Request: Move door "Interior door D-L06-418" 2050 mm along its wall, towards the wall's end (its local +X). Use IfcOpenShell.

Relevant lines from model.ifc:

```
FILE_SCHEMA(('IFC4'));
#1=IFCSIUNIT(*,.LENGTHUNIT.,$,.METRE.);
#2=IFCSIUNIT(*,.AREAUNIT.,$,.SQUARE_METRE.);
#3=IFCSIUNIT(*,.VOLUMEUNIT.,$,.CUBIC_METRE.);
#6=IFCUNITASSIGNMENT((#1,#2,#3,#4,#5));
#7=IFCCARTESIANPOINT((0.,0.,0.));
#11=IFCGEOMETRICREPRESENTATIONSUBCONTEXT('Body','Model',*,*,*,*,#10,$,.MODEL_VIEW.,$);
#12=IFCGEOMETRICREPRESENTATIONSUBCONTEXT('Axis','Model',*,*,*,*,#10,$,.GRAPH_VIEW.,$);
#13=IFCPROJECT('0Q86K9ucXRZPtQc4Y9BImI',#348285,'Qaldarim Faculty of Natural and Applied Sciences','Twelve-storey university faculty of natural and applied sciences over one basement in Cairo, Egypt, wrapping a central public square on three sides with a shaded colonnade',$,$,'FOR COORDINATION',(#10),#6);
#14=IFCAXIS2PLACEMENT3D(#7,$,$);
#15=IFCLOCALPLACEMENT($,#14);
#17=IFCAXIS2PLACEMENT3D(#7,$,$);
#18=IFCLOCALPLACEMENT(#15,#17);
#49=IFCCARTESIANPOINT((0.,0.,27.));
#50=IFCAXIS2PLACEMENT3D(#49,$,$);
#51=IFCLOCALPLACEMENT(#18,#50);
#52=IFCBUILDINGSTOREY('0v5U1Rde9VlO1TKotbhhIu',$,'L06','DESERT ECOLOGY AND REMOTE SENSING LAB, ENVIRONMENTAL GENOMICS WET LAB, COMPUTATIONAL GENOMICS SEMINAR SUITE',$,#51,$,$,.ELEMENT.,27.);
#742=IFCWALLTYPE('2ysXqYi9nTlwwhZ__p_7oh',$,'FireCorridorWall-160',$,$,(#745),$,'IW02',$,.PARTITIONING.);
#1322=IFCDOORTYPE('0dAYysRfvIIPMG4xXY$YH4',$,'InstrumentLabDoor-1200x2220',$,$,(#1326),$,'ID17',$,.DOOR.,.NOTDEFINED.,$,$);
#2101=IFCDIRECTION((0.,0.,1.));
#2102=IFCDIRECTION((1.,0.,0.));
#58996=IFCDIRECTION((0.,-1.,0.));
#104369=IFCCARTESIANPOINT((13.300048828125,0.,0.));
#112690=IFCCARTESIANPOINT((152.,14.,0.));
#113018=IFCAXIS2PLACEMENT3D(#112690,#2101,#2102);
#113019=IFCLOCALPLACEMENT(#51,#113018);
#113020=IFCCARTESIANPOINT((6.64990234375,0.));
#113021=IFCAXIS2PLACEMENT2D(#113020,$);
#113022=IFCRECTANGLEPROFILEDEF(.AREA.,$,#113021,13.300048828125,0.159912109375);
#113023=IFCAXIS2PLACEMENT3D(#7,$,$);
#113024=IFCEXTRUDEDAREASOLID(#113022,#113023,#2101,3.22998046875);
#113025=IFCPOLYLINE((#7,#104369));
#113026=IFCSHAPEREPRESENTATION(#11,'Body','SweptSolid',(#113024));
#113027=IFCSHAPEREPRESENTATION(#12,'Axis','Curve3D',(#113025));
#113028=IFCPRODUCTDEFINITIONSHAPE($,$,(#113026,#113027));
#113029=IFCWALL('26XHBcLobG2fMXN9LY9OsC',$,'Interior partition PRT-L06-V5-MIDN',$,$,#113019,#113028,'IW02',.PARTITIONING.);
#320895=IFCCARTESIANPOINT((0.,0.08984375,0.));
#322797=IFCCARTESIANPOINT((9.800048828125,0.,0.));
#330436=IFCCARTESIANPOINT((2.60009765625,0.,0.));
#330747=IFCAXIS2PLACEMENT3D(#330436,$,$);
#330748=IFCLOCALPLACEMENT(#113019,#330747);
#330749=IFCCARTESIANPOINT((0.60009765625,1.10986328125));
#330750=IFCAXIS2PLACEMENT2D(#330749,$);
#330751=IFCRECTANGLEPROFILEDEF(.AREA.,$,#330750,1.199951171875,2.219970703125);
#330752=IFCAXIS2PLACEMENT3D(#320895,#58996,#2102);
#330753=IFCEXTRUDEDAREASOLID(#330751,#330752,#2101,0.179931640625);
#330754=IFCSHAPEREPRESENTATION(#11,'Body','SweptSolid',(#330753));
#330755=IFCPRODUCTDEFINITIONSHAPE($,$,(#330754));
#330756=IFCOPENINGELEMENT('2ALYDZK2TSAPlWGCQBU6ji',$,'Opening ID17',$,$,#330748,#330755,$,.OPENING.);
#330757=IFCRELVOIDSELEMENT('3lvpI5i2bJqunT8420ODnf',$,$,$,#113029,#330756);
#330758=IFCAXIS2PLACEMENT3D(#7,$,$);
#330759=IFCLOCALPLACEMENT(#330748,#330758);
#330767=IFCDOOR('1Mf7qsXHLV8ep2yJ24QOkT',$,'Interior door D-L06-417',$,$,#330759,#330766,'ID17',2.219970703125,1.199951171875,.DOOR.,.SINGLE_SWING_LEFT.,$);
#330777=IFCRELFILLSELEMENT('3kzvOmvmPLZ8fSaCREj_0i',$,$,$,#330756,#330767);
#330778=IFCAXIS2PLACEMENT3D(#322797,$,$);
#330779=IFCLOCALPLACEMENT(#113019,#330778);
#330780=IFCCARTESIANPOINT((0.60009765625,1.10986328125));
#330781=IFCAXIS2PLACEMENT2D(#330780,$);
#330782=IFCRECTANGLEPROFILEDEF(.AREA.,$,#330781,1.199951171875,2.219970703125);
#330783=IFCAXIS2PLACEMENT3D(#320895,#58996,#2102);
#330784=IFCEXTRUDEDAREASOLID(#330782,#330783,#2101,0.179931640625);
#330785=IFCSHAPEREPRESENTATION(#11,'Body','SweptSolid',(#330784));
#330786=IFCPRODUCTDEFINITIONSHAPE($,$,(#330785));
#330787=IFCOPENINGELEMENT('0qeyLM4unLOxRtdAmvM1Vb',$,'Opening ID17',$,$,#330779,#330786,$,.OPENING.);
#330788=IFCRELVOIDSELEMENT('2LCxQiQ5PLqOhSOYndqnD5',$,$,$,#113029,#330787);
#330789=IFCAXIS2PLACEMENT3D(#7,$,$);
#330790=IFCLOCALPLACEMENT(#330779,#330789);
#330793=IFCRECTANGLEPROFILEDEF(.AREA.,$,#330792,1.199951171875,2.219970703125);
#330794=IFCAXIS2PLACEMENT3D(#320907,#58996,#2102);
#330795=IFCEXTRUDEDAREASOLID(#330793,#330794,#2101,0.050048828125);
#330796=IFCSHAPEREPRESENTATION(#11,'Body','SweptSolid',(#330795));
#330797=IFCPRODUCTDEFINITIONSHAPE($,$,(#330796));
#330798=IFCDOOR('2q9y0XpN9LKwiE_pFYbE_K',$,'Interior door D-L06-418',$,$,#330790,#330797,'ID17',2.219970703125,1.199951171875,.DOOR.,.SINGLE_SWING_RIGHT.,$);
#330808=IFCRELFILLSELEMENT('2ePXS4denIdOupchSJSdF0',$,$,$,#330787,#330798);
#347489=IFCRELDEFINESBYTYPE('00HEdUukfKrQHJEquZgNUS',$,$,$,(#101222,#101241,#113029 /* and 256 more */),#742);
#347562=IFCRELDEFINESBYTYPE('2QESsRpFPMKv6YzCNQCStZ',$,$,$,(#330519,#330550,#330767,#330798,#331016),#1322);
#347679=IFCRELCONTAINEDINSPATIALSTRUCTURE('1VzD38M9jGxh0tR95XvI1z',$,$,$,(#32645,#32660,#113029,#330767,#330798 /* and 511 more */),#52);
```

```python
import ifcopenshell
import ifcopenshell.api.geometry
import ifcopenshell.util.placement

model = ifcopenshell.open("model.ifc")

door = model.by_guid("2q9y0XpN9LKwiE_pFYbE_K")
opening = door.FillsVoids[0].RelatingOpeningElement
wall = opening.VoidsElements[0].RelatingBuildingElement

wall_matrix = ifcopenshell.util.placement.get_local_placement(wall.ObjectPlacement)
shift = wall_matrix[:3, 0] * 2.05
before = ifcopenshell.util.placement.get_local_placement(door.ObjectPlacement)[:3, 3].copy()

# The door is placed relative to its opening, so it follows when the opening moves.
matrix = ifcopenshell.util.placement.get_local_placement(opening.ObjectPlacement)
matrix[:3, 3] += shift
ifcopenshell.api.geometry.edit_object_placement(
    model, product=opening, matrix=matrix, is_si=False, should_transform_children=True
)

after = ifcopenshell.util.placement.get_local_placement(door.ObjectPlacement)[:3, 3]
print("door moved by", (after - before).round(3) + 0.0)

model.write("model-out.ifc")
```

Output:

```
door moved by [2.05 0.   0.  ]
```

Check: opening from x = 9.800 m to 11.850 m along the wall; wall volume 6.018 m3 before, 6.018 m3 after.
